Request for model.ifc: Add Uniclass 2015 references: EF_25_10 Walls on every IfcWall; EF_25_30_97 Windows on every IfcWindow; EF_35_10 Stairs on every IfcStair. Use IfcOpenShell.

First a look at what the model holds.

```python
import ifcopenshell

model = ifcopenshell.open("model.ifc")
print(model.schema)
print("classifications:", [c.Name for c in model.by_type("IfcClassification")])
for ifc_class in ("IfcDoor", "IfcRoof", "IfcStair", "IfcWall", "IfcWindow"):
    print(ifc_class, len(model.by_type(ifc_class)))
```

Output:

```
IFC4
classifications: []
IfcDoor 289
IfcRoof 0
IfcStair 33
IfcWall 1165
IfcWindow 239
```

```python
import ifcopenshell
import ifcopenshell.api.classification

model = ifcopenshell.open("model.ifc")

system = ifcopenshell.api.classification.add_classification(model, classification="Uniclass 2015")

codes = {
    "IfcWall": ("EF_25_10", "Walls"),
    "IfcWindow": ("EF_25_30_97", "Windows"),
    "IfcStair": ("EF_35_10", "Stairs"),
}
for ifc_class, (code, name) in codes.items():
    products = model.by_type(ifc_class)
    ifcopenshell.api.classification.add_reference(
        model, products=products, classification=system, identification=code, name=name
    )
    print(code, len(products))

model.write("model_edited.ifc")
```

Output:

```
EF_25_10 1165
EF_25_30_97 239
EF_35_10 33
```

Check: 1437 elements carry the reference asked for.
